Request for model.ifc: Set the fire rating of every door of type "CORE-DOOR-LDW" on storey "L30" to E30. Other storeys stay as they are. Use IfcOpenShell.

First a look at what the model holds.

```python
import ifcopenshell
import ifcopenshell.util.element

model = ifcopenshell.open("model.ifc")
print(model.schema)
storey = next(s for s in model.by_type("IfcBuildingStorey") if s.Name == "L30")
doors = [e for e in ifcopenshell.util.element.get_decomposition(storey) if e.is_a("IfcDoor")]
seen = {}
for e in doors:
    element_type = ifcopenshell.util.element.get_type(e)
    key = (element_type.Name if element_type != e and element_type else None, ifcopenshell.util.element.get_pset(e, "Pset_DoorCommon", "FireRating"))
    seen[key] = seen.get(key, 0) + 1
for (name, value), count in sorted(seen.items(), key=str):
    print(count, "x", name, "|", value)
```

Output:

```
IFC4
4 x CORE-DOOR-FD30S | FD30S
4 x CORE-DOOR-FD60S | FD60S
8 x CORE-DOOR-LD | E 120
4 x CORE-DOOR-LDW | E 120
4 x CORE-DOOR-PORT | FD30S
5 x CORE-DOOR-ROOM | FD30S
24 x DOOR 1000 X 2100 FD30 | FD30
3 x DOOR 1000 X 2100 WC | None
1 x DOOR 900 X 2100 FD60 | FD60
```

```python
import ifcopenshell
import ifcopenshell.api.pset
import ifcopenshell.util.element

model = ifcopenshell.open("model.ifc")

storey = next(s for s in model.by_type("IfcBuildingStorey") if s.Name == "L30")
doors = [e for e in ifcopenshell.util.element.get_decomposition(storey) if e.is_a("IfcDoor")]

count = 0
for e in doors:
    element_type = ifcopenshell.util.element.get_type(e)
    if element_type in (None, e) or element_type.Name != "CORE-DOOR-LDW":
        continue
    # add_pset returns the element's existing set when there is one.
    pset = ifcopenshell.api.pset.add_pset(model, product=e, name="Pset_DoorCommon")
    ifcopenshell.api.pset.edit_pset(model, pset=pset, properties={"FireRating": "E30"})
    count += 1

print(count, "doors updated")

model.write("model_edited.ifc")
```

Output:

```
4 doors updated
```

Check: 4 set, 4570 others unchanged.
